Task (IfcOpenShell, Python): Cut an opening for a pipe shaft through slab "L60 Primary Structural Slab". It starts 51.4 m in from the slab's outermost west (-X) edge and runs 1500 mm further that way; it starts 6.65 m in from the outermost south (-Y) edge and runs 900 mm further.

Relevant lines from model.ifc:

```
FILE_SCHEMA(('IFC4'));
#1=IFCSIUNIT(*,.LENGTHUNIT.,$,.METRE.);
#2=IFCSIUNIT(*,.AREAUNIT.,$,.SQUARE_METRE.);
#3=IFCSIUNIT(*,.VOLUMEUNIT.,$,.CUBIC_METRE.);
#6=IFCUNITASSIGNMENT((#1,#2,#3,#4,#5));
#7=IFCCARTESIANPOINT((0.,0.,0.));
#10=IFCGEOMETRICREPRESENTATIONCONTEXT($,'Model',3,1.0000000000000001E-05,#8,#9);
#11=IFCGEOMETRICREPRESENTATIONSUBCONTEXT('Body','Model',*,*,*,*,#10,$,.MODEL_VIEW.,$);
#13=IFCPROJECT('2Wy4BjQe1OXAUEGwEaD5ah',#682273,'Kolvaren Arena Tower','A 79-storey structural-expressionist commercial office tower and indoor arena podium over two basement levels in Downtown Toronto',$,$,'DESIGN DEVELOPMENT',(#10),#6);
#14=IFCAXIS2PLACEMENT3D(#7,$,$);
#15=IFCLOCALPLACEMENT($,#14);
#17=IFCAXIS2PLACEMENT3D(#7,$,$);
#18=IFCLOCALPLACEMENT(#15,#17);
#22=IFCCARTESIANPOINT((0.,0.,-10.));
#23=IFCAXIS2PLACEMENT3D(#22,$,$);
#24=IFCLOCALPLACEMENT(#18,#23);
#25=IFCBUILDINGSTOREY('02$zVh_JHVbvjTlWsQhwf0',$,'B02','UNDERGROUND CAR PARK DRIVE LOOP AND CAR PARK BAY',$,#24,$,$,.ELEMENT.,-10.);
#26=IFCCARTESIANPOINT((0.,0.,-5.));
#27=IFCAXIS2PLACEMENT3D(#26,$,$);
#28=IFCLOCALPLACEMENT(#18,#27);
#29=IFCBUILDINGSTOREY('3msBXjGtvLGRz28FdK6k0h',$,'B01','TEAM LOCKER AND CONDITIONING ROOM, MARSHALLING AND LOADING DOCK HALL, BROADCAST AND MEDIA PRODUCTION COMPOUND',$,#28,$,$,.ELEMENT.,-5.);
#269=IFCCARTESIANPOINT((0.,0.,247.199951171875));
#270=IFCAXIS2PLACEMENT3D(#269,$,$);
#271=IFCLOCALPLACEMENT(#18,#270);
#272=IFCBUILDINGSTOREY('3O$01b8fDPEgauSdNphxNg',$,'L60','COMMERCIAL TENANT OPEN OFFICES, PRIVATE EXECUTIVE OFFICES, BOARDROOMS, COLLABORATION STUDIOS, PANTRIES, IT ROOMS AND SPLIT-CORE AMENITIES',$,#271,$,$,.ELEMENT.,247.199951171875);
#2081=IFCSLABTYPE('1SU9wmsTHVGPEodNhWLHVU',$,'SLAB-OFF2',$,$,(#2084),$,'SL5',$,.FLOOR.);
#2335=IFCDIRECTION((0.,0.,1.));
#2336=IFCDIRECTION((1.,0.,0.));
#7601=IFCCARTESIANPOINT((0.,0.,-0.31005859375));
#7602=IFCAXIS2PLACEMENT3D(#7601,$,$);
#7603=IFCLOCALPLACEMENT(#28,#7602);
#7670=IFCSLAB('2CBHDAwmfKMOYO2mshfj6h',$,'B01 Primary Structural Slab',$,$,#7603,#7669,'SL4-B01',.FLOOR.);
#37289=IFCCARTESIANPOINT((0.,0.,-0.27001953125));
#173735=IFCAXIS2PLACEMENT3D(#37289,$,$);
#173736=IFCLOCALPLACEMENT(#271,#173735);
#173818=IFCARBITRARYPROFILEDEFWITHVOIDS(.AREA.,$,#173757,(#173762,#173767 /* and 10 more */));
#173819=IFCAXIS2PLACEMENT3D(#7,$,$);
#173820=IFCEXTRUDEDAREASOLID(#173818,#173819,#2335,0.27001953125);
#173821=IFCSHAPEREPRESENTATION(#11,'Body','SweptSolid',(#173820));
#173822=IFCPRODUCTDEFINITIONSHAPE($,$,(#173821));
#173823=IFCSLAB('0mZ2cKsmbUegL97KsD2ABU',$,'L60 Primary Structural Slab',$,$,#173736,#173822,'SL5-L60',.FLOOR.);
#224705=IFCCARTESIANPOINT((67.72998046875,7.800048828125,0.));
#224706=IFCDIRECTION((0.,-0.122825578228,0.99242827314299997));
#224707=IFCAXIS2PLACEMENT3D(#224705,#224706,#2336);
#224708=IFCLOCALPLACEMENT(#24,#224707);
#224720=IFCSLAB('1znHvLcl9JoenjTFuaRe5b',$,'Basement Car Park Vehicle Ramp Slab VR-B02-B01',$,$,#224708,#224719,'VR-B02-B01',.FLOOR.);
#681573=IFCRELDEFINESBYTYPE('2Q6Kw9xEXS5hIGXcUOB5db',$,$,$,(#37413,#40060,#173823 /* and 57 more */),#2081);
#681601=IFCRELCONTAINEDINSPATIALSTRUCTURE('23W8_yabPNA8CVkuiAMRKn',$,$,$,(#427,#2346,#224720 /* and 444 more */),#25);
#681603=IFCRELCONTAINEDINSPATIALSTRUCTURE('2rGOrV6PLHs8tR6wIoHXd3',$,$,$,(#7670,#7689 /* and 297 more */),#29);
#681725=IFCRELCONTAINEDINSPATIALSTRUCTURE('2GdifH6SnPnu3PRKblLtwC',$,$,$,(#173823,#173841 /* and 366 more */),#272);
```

```python
import numpy as np
import ifcopenshell
import ifcopenshell.api.feature
import ifcopenshell.api.geometry
import ifcopenshell.api.root
import ifcopenshell.geom
import ifcopenshell.util.placement
import ifcopenshell.util.representation
import ifcopenshell.util.shape
import ifcopenshell.util.unit

model = ifcopenshell.open("model.ifc")
unit_scale = ifcopenshell.util.unit.calculate_unit_scale(model)
settings = ifcopenshell.geom.settings()


def volume(element):
    """Net volume in cubic metres, openings subtracted."""
    shape = ifcopenshell.geom.create_shape(settings, element)
    return ifcopenshell.util.shape.get_volume(shape.geometry)


slab = model.by_id(173823)
before = volume(slab)

# Extent in the slab's own axes, in metres. The edges named are its -X and -Y sides.
slab_shape = ifcopenshell.geom.create_shape(settings, slab)
vertices = ifcopenshell.util.shape.get_vertices(slab_shape.geometry)
x_min, y_min, bottom = vertices.min(axis=0)
top = vertices[:, 2].max()

opening = ifcopenshell.api.root.create_entity(model, ifc_class="IfcOpeningElement", name="Pipe shaft opening", predefined_type="OPENING")
context = ifcopenshell.util.representation.get_context(model, "Model", "Body", "MODEL_VIEW")
width, depth = 1.5, 0.9
outline = [(0.0, 0.0), (width, 0.0), (width, depth), (0.0, depth), (0.0, 0.0)]
# Overshoot both faces by 50 mm so the cut is clean.
shape = ifcopenshell.api.geometry.add_slab_representation(
    model, context=context, depth=top - bottom + 0.1, polyline=outline
)
ifcopenshell.api.geometry.assign_representation(model, product=opening, representation=shape)

matrix = ifcopenshell.util.placement.get_local_placement(slab.ObjectPlacement)
matrix[:, 3] = matrix @ np.append(np.array([x_min + 51.4, y_min + 6.65, bottom - 0.05]) / unit_scale, 1.0)
ifcopenshell.api.geometry.edit_object_placement(model, product=opening, matrix=matrix, is_si=False)
ifcopenshell.api.feature.add_feature(model, feature=opening, element=slab)

after = volume(slab)

print(f"slab volume {before:.3f} -> {after:.3f} m3")

model.write("model_edited.ifc")
```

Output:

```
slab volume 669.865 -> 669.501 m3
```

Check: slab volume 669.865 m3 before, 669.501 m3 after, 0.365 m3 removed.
